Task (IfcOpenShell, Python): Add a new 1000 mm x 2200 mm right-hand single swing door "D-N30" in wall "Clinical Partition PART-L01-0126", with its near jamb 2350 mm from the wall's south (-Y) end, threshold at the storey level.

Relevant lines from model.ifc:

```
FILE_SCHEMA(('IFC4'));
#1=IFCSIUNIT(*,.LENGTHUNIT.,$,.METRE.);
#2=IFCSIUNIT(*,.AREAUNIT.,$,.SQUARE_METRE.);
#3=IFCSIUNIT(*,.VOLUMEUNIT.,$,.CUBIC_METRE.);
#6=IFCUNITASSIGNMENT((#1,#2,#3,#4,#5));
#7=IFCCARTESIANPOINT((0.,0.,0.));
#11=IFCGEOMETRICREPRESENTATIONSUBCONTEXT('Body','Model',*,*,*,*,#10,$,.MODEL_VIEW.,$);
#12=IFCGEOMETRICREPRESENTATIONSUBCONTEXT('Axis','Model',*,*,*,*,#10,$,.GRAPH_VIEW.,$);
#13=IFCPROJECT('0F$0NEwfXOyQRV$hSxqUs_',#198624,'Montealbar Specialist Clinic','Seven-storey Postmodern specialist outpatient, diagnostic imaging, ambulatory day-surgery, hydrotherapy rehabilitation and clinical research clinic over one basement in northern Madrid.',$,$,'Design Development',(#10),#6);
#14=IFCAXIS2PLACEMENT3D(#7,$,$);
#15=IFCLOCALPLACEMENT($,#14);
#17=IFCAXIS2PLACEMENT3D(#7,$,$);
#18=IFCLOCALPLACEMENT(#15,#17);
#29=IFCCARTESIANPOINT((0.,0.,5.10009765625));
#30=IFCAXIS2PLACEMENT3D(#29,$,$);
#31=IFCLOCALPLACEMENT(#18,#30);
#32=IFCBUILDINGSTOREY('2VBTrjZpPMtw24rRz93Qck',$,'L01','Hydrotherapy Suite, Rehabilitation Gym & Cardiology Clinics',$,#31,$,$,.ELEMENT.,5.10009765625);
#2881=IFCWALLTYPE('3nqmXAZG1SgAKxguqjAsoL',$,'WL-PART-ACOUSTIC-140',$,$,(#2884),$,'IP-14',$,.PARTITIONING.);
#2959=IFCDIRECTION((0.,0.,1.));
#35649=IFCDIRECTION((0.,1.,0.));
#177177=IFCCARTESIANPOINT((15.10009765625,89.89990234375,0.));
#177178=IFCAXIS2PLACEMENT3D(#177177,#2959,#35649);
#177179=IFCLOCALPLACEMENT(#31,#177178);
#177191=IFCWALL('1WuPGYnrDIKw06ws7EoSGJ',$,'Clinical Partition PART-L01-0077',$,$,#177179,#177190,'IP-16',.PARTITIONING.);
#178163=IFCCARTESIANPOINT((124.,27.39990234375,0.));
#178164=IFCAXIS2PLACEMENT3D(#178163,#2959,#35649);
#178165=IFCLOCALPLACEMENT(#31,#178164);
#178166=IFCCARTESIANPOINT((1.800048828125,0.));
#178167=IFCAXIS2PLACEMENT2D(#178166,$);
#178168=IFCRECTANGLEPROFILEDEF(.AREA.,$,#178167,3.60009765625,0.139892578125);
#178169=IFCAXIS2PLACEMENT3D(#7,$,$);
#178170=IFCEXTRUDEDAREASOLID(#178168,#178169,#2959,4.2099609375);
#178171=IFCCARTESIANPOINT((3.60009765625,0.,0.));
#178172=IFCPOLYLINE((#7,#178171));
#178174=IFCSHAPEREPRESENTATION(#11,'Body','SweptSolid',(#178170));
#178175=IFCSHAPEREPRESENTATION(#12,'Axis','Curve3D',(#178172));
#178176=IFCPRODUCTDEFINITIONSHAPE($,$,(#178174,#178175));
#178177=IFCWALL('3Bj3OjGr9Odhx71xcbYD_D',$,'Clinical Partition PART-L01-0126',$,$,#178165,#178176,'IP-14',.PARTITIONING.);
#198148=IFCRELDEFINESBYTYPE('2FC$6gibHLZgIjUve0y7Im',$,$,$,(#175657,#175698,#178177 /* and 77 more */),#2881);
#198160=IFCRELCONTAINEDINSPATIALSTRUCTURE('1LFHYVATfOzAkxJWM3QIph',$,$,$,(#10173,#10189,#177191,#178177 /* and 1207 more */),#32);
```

```python
import numpy as np
import ifcopenshell
import ifcopenshell.api.feature
import ifcopenshell.api.geometry
import ifcopenshell.api.root
import ifcopenshell.api.spatial
import ifcopenshell.geom
import ifcopenshell.util.element
import ifcopenshell.util.placement
import ifcopenshell.util.representation
import ifcopenshell.util.shape
import ifcopenshell.util.unit

model = ifcopenshell.open("model.ifc")
unit_scale = ifcopenshell.util.unit.calculate_unit_scale(model)
settings = ifcopenshell.geom.settings()


def volume(element):
    """Net volume in cubic metres, openings subtracted."""
    shape = ifcopenshell.geom.create_shape(settings, element)
    return ifcopenshell.util.shape.get_volume(shape.geometry)


wall = model.by_guid("3Bj3OjGr9Odhx71xcbYD_D")
storey = ifcopenshell.util.element.get_container(wall, ifc_class="IfcBuildingStorey")
context = ifcopenshell.util.representation.get_context(model, "Model", "Body", "MODEL_VIEW")
before = volume(wall)

width, height, from_end, sill = 1, 2.2, 2.35, 0.0  # metres

# The wall runs along its own X axis, and the end named is its -X end.
wall_shape = ifcopenshell.geom.create_shape(settings, wall)
x, y, z = ifcopenshell.util.shape.get_vertices(wall_shape.geometry).T
start = x.min() + from_end
face, thickness = float(y.min()), float(y.max() - y.min())
wall_matrix = ifcopenshell.util.placement.get_local_placement(wall.ObjectPlacement)
level = ifcopenshell.util.placement.get_local_placement(storey.ObjectPlacement)[2, 3]


def in_wall(x, y):
    """Placement at x, y metres in the wall's axes, at sill height."""
    matrix = wall_matrix.copy()
    matrix[:, 3] = wall_matrix @ np.array([x / unit_scale, y / unit_scale, 0.0, 1.0])
    matrix[2, 3] = level + sill / unit_scale
    return matrix


# Opening: a box that overshoots both wall faces by 50 mm.
opening = ifcopenshell.api.root.create_entity(model, ifc_class="IfcOpeningElement", predefined_type="OPENING")
box = ifcopenshell.api.geometry.add_wall_representation(
    model, context=context, length=width, height=height, thickness=thickness + 0.1
)
ifcopenshell.api.geometry.assign_representation(model, product=opening, representation=box)
ifcopenshell.api.geometry.edit_object_placement(model, product=opening, matrix=in_wall(start, face - 0.05), is_si=False)
ifcopenshell.api.feature.add_feature(model, feature=opening, element=wall)

door = ifcopenshell.api.root.create_entity(model, ifc_class="IfcDoor", name="D-N30", predefined_type="DOOR")
door.OverallWidth, door.OverallHeight = width / unit_scale, height / unit_scale
door.OperationType = "SINGLE_SWING_RIGHT"
body = ifcopenshell.api.geometry.add_door_representation(
    model,
    context=context,
    overall_width=door.OverallWidth,
    overall_height=door.OverallHeight,
    operation_type="SINGLE_SWING_RIGHT",
    lining_properties={"LiningDepth": thickness / unit_scale, "ThresholdDepth": thickness / unit_scale},
)
ifcopenshell.api.geometry.assign_representation(model, product=door, representation=body)
ifcopenshell.api.spatial.assign_container(model, products=[door], relating_structure=storey)
ifcopenshell.api.feature.add_filling(model, opening=opening, element=door)

# The lining spans the wall, so the door starts at the wall face.
ifcopenshell.api.geometry.edit_object_placement(model, product=door, matrix=in_wall(start, face), is_si=False)

after = volume(wall)

print(f"wall volume {before:.3f} -> {after:.3f} m3")

model.write("model_edited.ifc")
```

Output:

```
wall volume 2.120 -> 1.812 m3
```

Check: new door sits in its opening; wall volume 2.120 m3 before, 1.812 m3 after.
